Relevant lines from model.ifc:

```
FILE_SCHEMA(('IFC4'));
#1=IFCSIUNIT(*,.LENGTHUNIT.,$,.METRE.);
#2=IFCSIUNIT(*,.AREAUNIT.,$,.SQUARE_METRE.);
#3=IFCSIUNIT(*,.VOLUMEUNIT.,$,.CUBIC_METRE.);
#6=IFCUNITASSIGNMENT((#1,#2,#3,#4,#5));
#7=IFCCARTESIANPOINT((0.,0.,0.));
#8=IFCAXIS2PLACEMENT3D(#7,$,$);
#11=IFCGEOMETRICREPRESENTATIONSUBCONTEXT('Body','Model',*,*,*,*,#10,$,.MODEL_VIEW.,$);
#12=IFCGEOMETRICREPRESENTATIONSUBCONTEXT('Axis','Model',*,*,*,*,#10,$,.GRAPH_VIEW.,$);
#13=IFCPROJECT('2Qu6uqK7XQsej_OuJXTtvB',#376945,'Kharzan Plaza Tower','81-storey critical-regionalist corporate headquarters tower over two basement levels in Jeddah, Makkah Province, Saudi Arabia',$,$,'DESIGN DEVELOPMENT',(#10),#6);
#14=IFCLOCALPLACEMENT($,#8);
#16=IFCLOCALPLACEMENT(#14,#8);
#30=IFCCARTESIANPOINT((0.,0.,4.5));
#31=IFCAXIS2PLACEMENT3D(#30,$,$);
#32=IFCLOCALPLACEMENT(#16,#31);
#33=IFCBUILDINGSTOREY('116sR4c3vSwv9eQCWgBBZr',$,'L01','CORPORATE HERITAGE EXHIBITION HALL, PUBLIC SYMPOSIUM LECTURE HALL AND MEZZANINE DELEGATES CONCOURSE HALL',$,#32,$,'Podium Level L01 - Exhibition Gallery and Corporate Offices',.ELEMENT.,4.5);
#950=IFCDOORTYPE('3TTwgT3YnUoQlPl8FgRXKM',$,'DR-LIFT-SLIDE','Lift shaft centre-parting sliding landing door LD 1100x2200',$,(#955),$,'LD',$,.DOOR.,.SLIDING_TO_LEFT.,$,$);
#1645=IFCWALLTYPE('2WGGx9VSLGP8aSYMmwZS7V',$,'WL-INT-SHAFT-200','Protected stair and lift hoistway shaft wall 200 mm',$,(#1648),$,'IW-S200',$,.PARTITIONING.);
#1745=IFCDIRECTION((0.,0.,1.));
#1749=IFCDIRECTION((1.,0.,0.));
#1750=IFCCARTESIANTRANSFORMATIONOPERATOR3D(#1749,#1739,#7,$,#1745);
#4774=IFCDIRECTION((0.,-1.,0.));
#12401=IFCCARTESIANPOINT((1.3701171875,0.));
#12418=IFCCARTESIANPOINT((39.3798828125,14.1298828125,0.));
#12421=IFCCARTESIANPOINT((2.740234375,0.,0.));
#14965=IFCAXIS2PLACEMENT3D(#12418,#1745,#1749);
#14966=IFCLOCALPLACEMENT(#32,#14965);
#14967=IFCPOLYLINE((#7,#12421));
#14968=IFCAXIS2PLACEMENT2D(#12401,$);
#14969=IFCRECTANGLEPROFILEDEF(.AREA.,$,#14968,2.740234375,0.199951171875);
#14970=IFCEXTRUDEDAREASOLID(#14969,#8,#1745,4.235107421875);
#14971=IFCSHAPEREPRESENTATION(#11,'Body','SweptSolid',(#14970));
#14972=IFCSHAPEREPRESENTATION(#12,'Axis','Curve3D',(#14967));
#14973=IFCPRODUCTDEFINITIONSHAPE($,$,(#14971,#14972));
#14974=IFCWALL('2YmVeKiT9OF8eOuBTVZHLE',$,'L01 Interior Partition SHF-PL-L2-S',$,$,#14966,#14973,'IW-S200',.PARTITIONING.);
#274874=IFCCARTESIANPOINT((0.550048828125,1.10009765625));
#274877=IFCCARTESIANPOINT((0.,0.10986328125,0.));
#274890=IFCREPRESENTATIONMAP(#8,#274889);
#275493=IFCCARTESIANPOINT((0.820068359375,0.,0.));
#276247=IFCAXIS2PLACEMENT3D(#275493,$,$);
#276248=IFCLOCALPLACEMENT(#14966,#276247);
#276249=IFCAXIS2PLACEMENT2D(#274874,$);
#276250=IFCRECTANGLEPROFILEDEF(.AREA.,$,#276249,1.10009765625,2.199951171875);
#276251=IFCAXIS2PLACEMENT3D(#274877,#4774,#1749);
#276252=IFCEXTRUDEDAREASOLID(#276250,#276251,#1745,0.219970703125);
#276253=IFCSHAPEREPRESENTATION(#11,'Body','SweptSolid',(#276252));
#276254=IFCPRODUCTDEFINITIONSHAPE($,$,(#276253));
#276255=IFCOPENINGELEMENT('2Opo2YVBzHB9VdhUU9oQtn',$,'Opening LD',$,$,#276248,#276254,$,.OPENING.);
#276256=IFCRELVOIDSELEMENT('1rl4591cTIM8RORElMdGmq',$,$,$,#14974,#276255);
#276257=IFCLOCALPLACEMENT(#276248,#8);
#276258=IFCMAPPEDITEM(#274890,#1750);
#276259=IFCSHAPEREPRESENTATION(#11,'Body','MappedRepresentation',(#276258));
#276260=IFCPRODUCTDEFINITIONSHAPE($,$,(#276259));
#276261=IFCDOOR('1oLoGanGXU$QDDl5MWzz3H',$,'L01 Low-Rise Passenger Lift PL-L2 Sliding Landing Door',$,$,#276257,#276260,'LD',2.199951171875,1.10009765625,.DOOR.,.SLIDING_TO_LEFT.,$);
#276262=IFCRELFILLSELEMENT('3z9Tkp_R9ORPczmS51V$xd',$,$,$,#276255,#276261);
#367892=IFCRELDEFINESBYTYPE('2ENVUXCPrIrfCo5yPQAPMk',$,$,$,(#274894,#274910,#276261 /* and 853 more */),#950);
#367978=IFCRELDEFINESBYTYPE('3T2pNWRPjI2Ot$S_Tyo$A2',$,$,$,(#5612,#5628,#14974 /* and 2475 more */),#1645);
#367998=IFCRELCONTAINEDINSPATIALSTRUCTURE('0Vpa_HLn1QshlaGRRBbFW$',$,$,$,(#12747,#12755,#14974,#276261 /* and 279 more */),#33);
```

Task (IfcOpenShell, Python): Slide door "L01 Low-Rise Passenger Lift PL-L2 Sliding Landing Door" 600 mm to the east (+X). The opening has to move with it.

```python
import ifcopenshell
import ifcopenshell.api.geometry
import ifcopenshell.util.placement
import ifcopenshell.util.unit

model = ifcopenshell.open("model.ifc")
unit_scale = ifcopenshell.util.unit.calculate_unit_scale(model)

door = model.by_guid("1oLoGanGXU$QDDl5MWzz3H")
opening = door.FillsVoids[0].RelatingOpeningElement
wall = opening.VoidsElements[0].RelatingBuildingElement

wall_matrix = ifcopenshell.util.placement.get_local_placement(wall.ObjectPlacement)
shift = wall_matrix[:3, 0] * 0.6 / unit_scale
before = ifcopenshell.util.placement.get_local_placement(door.ObjectPlacement)[:3, 3].copy()

# The door is placed relative to its opening, so it follows when the opening moves.
matrix = ifcopenshell.util.placement.get_local_placement(opening.ObjectPlacement)
matrix[:3, 3] += shift
ifcopenshell.api.geometry.edit_object_placement(
    model, product=opening, matrix=matrix, is_si=False, should_transform_children=True
)

after = ifcopenshell.util.placement.get_local_placement(door.ObjectPlacement)[:3, 3]
print("door moved by", (after - before).round(3) + 0.0)

model.write("model_v2.ifc")
```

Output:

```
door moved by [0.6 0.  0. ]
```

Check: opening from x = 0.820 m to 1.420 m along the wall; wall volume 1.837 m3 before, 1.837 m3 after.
